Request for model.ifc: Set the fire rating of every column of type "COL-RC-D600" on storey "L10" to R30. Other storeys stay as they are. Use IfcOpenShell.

First a look at what the model holds.

```python
import ifcopenshell
import ifcopenshell.util.element

model = ifcopenshell.open("model.ifc")
print(model.schema)
storey = next(s for s in model.by_type("IfcBuildingStorey") if s.Name == "L10")
columns = [e for e in ifcopenshell.util.element.get_decomposition(storey) if e.is_a("IfcColumn")]
seen = {}
for e in columns:
    element_type = ifcopenshell.util.element.get_type(e)
    key = (element_type.Name if element_type != e and element_type else None, ifcopenshell.util.element.get_pset(e, "Pset_ColumnCommon", "FireRating"))
    seen[key] = seen.get(key, 0) + 1
for (name, value), count in sorted(seen.items(), key=str):
    print(count, "x", name, "|", value)
```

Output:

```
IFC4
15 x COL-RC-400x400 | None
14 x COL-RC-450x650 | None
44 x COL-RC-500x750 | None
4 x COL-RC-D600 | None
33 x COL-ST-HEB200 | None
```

```python
import ifcopenshell
import ifcopenshell.api.pset
import ifcopenshell.util.element

model = ifcopenshell.open("model.ifc")

storey = next(s for s in model.by_type("IfcBuildingStorey") if s.Name == "L10")
columns = [e for e in ifcopenshell.util.element.get_decomposition(storey) if e.is_a("IfcColumn")]

count = 0
for e in columns:
    element_type = ifcopenshell.util.element.get_type(e)
    if element_type in (None, e) or element_type.Name != "COL-RC-D600":
        continue
    # add_pset returns the element's existing set when there is one.
    pset = ifcopenshell.api.pset.add_pset(model, product=e, name="Pset_ColumnCommon")
    ifcopenshell.api.pset.edit_pset(model, pset=pset, properties={"FireRating": "R30"})
    count += 1

print(count, "columns updated")

model.write("model_edited.ifc")
```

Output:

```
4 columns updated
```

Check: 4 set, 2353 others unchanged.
